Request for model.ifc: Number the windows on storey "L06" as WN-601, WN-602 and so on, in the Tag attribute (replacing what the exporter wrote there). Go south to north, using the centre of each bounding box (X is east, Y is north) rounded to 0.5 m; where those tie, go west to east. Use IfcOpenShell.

First a look at what the model holds.

```python
import ifcopenshell
import ifcopenshell.util.element
import ifcopenshell.util.placement

model = ifcopenshell.open("model.ifc")
print(model.schema)
storey = next(s for s in model.by_type("IfcBuildingStorey") if s.Name == "L06")
windows = [e for e in ifcopenshell.util.element.get_decomposition(storey) if e.is_a("IfcWindow")]
for e in sorted(windows, key=lambda e: e.id()):
    origin = ifcopenshell.util.placement.get_local_placement(e.ObjectPlacement)[:3, 3]
    print(e.id(), e.Tag, e.Name, origin.round(2) + 0.0, sep=" | ")
```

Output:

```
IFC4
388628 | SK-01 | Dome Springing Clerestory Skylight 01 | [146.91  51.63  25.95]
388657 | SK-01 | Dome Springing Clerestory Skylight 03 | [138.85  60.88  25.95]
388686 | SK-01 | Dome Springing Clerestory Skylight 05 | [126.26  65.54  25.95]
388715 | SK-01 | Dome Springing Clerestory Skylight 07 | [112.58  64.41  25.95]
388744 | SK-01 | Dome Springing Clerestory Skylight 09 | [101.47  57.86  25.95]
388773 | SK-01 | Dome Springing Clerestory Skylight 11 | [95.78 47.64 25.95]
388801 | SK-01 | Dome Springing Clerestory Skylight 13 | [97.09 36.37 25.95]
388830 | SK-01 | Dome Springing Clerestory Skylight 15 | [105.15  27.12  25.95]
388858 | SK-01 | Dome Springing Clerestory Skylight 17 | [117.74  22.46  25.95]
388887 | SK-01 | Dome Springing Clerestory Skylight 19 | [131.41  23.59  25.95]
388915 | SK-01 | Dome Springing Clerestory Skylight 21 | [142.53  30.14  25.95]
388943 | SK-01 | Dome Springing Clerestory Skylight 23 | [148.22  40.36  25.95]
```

```python
import ifcopenshell
import ifcopenshell.geom
import ifcopenshell.util.element
import ifcopenshell.util.shape

model = ifcopenshell.open("model.ifc")
settings = ifcopenshell.geom.settings()
settings.set("use-world-coords", True)


def centre(element):
    shape = ifcopenshell.geom.create_shape(settings, element)
    return ifcopenshell.util.shape.get_bbox_centroid(shape.geometry)


storey = next(s for s in model.by_type("IfcBuildingStorey") if s.Name == "L06")
windows = [e for e in ifcopenshell.util.element.get_decomposition(storey) if e.is_a("IfcWindow")]

# Insertion points can sit at a corner or the storey origin, so sort by the geometry (in metres).
centres = {e: centre(e) for e in windows}
windows.sort(key=lambda e: (round(centres[e][1] / 0.5), centres[e][0]))

for i, e in enumerate(windows, start=1):
    number = f"WN-6{i:02d}"
    e.Tag = number
    print(e.id(), number)

model.write("model_rev.ifc")
```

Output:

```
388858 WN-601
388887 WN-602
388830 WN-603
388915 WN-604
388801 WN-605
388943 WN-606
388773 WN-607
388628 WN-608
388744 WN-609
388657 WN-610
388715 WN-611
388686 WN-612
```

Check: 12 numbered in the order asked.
